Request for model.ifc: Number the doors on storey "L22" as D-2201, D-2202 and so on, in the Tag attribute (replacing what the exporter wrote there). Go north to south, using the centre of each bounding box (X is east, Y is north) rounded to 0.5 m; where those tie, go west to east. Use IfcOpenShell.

First a look at what the model holds.

```python
import ifcopenshell
import ifcopenshell.util.element
import ifcopenshell.util.placement

model = ifcopenshell.open("model.ifc")
print(model.schema)
storey = next(s for s in model.by_type("IfcBuildingStorey") if s.Name == "L22")
doors = [e for e in ifcopenshell.util.element.get_decomposition(storey) if e.is_a("IfcDoor")]
for e in sorted(doors, key=lambda e: e.id()):
    origin = ifcopenshell.util.placement.get_local_placement(e.ObjectPlacement)[:3, 3]
    print(e.id(), e.Tag, e.Name, origin.round(2) + 0.0, sep=" | ")
```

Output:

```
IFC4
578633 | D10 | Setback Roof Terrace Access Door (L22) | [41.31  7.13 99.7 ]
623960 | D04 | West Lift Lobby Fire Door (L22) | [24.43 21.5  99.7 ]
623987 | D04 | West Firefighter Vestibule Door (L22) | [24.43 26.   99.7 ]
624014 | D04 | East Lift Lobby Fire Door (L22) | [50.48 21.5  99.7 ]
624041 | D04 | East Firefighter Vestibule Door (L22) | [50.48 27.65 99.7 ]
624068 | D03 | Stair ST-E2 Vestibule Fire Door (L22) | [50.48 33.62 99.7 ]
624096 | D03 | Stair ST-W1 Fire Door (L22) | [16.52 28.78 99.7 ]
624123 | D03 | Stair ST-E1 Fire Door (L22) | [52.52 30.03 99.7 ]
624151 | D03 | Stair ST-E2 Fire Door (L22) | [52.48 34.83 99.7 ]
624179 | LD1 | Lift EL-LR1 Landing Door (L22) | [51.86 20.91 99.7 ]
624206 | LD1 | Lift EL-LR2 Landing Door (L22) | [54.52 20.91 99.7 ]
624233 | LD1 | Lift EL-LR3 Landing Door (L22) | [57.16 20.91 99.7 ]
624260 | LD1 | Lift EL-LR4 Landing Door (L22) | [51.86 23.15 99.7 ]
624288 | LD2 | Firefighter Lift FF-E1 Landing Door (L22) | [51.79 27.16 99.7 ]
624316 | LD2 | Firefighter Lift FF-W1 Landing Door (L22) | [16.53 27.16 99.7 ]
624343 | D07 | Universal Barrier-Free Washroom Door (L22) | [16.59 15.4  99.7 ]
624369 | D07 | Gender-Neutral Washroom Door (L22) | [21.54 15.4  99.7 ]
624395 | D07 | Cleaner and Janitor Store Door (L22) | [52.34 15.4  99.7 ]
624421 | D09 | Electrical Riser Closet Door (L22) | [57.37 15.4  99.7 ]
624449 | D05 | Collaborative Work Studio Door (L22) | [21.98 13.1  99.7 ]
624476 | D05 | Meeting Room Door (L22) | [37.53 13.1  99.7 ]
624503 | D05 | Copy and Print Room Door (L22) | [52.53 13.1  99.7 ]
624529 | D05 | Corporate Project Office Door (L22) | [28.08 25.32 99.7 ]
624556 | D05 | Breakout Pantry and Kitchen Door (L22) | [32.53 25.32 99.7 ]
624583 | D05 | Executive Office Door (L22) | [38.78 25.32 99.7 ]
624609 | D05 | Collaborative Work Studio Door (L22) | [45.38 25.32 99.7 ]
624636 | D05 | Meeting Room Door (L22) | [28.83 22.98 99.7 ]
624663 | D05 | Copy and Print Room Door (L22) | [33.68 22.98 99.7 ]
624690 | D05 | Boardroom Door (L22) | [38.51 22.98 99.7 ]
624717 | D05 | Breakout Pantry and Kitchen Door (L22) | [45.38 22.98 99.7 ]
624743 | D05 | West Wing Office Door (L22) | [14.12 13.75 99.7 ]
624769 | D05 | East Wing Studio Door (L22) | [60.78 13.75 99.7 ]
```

```python
import ifcopenshell
import ifcopenshell.geom
import ifcopenshell.util.element
import ifcopenshell.util.shape

model = ifcopenshell.open("model.ifc")
settings = ifcopenshell.geom.settings()
settings.set("use-world-coords", True)


def centre(element):
    shape = ifcopenshell.geom.create_shape(settings, element)
    return ifcopenshell.util.shape.get_bbox_centroid(shape.geometry)


storey = next(s for s in model.by_type("IfcBuildingStorey") if s.Name == "L22")
doors = [e for e in ifcopenshell.util.element.get_decomposition(storey) if e.is_a("IfcDoor")]

# Insertion points can sit at a corner or the storey origin, so sort by the geometry (in metres).
centres = {e: centre(e) for e in doors}
doors.sort(key=lambda e: (-round(centres[e][1] / 0.5), centres[e][0]))

for i, e in enumerate(doors, start=1):
    number = f"D-22{i:02d}"
    e.Tag = number
    print(e.id(), number)

model.write("model_v2.ifc")
```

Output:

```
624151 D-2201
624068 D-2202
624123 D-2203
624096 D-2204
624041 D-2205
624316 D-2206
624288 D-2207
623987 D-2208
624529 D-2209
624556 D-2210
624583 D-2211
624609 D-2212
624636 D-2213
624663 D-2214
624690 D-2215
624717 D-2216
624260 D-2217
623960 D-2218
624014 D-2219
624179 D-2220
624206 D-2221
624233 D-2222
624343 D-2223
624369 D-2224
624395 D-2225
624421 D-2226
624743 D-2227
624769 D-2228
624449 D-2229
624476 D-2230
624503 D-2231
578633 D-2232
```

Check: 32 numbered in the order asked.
